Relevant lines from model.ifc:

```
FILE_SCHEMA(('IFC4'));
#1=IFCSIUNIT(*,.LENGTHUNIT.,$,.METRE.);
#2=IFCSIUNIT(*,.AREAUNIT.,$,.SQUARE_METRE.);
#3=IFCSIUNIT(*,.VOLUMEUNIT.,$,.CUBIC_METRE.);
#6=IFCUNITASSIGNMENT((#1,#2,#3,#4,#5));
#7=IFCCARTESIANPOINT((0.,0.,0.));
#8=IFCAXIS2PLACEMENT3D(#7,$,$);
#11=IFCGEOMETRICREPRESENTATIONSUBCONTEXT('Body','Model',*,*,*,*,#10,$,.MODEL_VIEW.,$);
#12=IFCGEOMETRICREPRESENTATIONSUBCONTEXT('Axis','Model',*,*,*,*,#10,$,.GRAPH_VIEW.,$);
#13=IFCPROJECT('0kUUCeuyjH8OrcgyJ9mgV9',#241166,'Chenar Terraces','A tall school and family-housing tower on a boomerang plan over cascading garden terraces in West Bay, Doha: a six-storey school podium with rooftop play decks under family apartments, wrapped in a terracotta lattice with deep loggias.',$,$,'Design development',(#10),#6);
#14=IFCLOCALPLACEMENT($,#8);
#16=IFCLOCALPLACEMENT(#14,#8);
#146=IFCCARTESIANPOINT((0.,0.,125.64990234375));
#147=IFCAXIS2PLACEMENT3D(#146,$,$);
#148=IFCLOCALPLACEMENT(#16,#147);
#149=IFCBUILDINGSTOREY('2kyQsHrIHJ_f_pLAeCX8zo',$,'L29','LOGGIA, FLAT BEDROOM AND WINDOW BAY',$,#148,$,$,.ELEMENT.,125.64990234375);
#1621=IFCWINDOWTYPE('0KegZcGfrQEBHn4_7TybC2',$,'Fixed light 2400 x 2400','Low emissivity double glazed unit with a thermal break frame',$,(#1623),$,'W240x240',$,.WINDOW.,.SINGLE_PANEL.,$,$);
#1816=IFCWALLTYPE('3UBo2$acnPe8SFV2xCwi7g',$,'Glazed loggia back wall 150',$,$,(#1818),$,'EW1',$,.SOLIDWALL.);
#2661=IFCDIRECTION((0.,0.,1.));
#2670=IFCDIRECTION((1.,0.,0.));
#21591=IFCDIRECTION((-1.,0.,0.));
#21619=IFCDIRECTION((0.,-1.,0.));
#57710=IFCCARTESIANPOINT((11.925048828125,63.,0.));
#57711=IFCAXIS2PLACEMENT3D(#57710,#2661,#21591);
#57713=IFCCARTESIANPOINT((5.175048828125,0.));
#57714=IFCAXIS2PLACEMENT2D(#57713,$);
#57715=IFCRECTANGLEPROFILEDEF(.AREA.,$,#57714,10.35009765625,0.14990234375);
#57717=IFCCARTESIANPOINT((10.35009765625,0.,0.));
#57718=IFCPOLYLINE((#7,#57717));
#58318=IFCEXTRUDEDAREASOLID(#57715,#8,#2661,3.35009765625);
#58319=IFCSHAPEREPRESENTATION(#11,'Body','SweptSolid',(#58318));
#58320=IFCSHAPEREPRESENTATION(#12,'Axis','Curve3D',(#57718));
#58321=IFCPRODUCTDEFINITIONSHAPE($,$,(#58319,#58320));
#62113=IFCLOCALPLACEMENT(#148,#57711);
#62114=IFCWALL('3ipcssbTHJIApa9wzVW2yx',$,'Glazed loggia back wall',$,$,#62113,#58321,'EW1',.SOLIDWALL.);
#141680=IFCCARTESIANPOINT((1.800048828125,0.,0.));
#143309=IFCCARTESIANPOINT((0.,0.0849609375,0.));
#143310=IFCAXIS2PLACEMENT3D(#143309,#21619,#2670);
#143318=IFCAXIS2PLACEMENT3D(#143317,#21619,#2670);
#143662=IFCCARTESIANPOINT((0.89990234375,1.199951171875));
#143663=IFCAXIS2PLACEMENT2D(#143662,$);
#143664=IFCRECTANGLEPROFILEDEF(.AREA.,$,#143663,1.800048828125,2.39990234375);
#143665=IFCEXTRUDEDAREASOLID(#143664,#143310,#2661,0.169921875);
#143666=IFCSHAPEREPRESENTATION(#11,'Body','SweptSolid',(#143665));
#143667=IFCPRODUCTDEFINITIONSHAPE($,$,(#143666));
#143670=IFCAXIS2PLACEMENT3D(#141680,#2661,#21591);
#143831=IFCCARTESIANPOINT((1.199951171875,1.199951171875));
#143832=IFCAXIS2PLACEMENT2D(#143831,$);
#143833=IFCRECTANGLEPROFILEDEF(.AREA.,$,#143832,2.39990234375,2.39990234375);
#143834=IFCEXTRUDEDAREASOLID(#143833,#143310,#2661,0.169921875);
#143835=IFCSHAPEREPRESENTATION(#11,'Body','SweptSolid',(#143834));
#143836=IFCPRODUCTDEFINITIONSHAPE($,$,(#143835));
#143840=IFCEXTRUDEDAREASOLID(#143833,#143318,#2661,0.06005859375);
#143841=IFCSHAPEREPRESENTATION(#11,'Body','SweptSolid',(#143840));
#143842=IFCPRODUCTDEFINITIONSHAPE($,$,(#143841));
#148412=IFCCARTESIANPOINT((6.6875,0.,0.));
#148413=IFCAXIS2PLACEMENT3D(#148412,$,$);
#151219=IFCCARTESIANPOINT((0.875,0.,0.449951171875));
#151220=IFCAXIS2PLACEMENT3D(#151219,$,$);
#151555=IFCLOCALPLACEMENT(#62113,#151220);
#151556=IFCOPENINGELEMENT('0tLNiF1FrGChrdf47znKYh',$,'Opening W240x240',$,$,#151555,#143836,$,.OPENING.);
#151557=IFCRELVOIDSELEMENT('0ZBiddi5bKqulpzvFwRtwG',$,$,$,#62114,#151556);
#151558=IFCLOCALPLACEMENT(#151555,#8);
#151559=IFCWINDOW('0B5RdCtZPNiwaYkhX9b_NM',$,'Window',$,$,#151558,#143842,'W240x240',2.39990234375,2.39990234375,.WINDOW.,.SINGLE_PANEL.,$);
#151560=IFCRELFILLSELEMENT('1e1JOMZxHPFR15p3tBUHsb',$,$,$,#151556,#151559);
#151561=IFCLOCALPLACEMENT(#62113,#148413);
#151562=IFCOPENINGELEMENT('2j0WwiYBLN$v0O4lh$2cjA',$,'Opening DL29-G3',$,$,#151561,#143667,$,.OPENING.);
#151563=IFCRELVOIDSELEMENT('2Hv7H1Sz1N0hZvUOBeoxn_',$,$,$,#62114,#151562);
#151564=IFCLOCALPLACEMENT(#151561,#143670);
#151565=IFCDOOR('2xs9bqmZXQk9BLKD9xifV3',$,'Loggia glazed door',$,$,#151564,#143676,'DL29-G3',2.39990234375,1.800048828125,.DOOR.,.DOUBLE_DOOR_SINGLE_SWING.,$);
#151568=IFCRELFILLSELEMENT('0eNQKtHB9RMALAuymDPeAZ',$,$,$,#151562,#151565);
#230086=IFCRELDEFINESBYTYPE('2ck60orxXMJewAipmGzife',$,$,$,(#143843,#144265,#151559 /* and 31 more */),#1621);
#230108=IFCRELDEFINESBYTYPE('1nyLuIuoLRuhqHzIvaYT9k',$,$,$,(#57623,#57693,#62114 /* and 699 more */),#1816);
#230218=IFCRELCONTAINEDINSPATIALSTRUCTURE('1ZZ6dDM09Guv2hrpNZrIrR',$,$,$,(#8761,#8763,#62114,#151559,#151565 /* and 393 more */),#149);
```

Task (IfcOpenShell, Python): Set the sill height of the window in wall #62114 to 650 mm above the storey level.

```python
import numpy as np
import ifcopenshell
import ifcopenshell.api.geometry
import ifcopenshell.geom
import ifcopenshell.util.element
import ifcopenshell.util.placement
import ifcopenshell.util.shape
import ifcopenshell.util.unit

model = ifcopenshell.open("model.ifc")
unit_scale = ifcopenshell.util.unit.calculate_unit_scale(model)

window = model.by_id(151559)
opening = window.FillsVoids[0].RelatingOpeningElement
storey = ifcopenshell.util.element.get_container(window, ifc_class="IfcBuildingStorey")
level = ifcopenshell.util.placement.get_local_placement(storey.ObjectPlacement)[2, 3]

# The opening's origin need not be at the sill, so measure its lowest point.
shape = ifcopenshell.geom.create_shape(ifcopenshell.geom.settings(), opening)
bottom = ifcopenshell.util.shape.get_shape_bottom_elevation(shape, shape.geometry) / unit_scale
dz = level + 0.65 / unit_scale - bottom

shift = np.array([0.0, 0.0, dz])
# The window is placed relative to its opening, so it follows when the opening moves.
matrix = ifcopenshell.util.placement.get_local_placement(opening.ObjectPlacement)
matrix[:3, 3] += shift
ifcopenshell.api.geometry.edit_object_placement(
    model, product=opening, matrix=matrix, is_si=False, should_transform_children=True
)

print(f"moved by {dz * unit_scale:+.3f} m")

model.write("model_updated.ifc")
```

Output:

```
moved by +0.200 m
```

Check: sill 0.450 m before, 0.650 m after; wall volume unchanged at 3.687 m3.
